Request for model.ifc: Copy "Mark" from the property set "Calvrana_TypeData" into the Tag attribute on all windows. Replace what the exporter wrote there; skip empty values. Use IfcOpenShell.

First a look at what the model holds.

```python
import ifcopenshell
import ifcopenshell.util.element

model = ifcopenshell.open("model.ifc")
print(model.schema)
windows = model.by_type("IfcWindow")
print(len(windows), "windows")
for e in windows[:8]:
    source = ifcopenshell.util.element.get_pset(e, "Calvrana_TypeData", "Mark")
    target = e.Tag
    print(e.id(), repr(source), repr(target), sep=" | ")
```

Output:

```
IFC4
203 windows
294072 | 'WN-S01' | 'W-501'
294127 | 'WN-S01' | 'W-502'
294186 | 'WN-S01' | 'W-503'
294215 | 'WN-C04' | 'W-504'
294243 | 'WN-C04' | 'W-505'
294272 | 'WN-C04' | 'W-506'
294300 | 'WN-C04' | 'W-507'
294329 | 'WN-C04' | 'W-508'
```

```python
import ifcopenshell
import ifcopenshell.util.element

model = ifcopenshell.open("model.ifc")

count = 0
for e in model.by_type("IfcWindow"):
    value = ifcopenshell.util.element.get_pset(e, "Calvrana_TypeData", "Mark")
    current = e.Tag
    if not value or not value.strip() or current == value:
        continue
    e.Tag = value
    count += 1

print(count, "windows updated")

model.write("model_edited.ifc")
```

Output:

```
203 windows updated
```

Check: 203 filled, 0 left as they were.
